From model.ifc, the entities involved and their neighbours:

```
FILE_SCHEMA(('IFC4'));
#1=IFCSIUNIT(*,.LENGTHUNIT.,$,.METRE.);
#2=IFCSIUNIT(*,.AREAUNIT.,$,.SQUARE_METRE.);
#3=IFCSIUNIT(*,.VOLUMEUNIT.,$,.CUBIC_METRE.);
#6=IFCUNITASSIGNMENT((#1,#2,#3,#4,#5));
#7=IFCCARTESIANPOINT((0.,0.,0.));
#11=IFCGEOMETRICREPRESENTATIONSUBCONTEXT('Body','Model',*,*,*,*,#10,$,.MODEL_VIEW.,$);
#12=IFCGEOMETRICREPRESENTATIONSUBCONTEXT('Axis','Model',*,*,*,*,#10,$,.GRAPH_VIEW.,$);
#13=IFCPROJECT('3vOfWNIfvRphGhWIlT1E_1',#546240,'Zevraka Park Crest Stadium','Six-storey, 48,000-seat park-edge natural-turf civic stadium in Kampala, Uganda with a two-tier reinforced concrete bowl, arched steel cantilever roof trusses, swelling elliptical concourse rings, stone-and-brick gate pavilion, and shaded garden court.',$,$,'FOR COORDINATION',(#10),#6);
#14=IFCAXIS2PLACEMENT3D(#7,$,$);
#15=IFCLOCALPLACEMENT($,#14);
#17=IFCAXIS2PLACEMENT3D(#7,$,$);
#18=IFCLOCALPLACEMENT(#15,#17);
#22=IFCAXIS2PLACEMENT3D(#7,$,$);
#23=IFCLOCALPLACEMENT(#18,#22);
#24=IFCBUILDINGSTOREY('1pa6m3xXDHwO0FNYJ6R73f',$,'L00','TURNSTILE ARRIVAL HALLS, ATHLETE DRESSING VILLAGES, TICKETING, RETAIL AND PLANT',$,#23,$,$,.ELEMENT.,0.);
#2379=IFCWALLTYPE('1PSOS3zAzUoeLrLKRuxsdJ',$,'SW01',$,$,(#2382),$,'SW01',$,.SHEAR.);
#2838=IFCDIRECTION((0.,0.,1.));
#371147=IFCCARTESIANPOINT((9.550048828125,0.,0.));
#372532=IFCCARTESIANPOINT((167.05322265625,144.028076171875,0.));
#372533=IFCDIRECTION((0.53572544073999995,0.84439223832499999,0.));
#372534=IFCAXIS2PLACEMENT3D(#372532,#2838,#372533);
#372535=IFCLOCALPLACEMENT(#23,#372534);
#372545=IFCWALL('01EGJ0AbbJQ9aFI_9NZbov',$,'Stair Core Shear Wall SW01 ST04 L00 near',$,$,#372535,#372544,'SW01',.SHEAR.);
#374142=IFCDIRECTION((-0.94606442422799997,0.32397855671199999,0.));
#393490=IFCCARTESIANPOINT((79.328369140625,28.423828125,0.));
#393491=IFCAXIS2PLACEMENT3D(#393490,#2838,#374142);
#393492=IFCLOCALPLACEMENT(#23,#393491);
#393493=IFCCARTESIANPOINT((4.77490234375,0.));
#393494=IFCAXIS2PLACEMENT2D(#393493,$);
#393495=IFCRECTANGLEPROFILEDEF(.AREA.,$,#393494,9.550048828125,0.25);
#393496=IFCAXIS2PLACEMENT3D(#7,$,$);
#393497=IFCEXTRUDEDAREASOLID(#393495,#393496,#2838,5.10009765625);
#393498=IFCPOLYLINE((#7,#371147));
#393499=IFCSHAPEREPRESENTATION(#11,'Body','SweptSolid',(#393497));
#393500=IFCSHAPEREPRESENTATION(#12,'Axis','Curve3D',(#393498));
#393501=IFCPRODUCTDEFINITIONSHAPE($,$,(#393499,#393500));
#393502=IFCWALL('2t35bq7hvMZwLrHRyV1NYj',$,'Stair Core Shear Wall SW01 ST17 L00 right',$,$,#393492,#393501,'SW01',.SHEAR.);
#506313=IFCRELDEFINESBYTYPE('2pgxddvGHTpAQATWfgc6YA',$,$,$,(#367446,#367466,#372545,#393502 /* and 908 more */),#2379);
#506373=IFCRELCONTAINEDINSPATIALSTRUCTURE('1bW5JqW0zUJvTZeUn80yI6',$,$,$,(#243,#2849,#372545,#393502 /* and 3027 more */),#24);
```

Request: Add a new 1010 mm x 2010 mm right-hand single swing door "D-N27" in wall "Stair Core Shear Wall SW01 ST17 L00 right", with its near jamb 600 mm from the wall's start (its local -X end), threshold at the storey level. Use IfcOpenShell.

```python
import numpy as np
import ifcopenshell
import ifcopenshell.api.feature
import ifcopenshell.api.geometry
import ifcopenshell.api.root
import ifcopenshell.api.spatial
import ifcopenshell.geom
import ifcopenshell.util.element
import ifcopenshell.util.placement
import ifcopenshell.util.representation
import ifcopenshell.util.shape
import ifcopenshell.util.unit

model = ifcopenshell.open("model.ifc")
unit_scale = ifcopenshell.util.unit.calculate_unit_scale(model)
settings = ifcopenshell.geom.settings()


def volume(element):
    """Net volume in cubic metres, openings subtracted."""
    shape = ifcopenshell.geom.create_shape(settings, element)
    return ifcopenshell.util.shape.get_volume(shape.geometry)


wall = model.by_id(393502)
storey = ifcopenshell.util.element.get_container(wall, ifc_class="IfcBuildingStorey")
context = ifcopenshell.util.representation.get_context(model, "Model", "Body", "MODEL_VIEW")
before = volume(wall)

width, height, from_end, sill = 1.01, 2.01, 0.6, 0.0  # metres

# The wall runs along its own X axis, and the end named is its -X end.
wall_shape = ifcopenshell.geom.create_shape(settings, wall)
x, y, z = ifcopenshell.util.shape.get_vertices(wall_shape.geometry).T
start = x.min() + from_end
face, thickness = float(y.min()), float(y.max() - y.min())
wall_matrix = ifcopenshell.util.placement.get_local_placement(wall.ObjectPlacement)
level = ifcopenshell.util.placement.get_local_placement(storey.ObjectPlacement)[2, 3]


def in_wall(x, y):
    """Placement at x, y metres in the wall's axes, at sill height."""
    matrix = wall_matrix.copy()
    matrix[:, 3] = wall_matrix @ np.array([x / unit_scale, y / unit_scale, 0.0, 1.0])
    matrix[2, 3] = level + sill / unit_scale
    return matrix


# Opening: a box that overshoots both wall faces by 50 mm.
opening = ifcopenshell.api.root.create_entity(model, ifc_class="IfcOpeningElement", predefined_type="OPENING")
box = ifcopenshell.api.geometry.add_wall_representation(
    model, context=context, length=width, height=height, thickness=thickness + 0.1
)
ifcopenshell.api.geometry.assign_representation(model, product=opening, representation=box)
ifcopenshell.api.geometry.edit_object_placement(model, product=opening, matrix=in_wall(start, face - 0.05), is_si=False)
ifcopenshell.api.feature.add_feature(model, feature=opening, element=wall)

door = ifcopenshell.api.root.create_entity(model, ifc_class="IfcDoor", name="D-N27", predefined_type="DOOR")
door.OverallWidth, door.OverallHeight = width / unit_scale, height / unit_scale
door.OperationType = "SINGLE_SWING_RIGHT"
body = ifcopenshell.api.geometry.add_door_representation(
    model,
    context=context,
    overall_width=door.OverallWidth,
    overall_height=door.OverallHeight,
    operation_type="SINGLE_SWING_RIGHT",
    lining_properties={"LiningDepth": thickness / unit_scale, "ThresholdDepth": thickness / unit_scale},
)
ifcopenshell.api.geometry.assign_representation(model, product=door, representation=body)
ifcopenshell.api.spatial.assign_container(model, products=[door], relating_structure=storey)
ifcopenshell.api.feature.add_filling(model, opening=opening, element=door)

# The lining spans the wall, so the door starts at the wall face.
ifcopenshell.api.geometry.edit_object_placement(model, product=door, matrix=in_wall(start, face), is_si=False)

after = volume(wall)

print(f"wall volume {before:.3f} -> {after:.3f} m3")

model.write("model-out.ifc")
```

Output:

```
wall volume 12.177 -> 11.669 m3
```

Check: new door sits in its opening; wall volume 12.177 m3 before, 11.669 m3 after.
